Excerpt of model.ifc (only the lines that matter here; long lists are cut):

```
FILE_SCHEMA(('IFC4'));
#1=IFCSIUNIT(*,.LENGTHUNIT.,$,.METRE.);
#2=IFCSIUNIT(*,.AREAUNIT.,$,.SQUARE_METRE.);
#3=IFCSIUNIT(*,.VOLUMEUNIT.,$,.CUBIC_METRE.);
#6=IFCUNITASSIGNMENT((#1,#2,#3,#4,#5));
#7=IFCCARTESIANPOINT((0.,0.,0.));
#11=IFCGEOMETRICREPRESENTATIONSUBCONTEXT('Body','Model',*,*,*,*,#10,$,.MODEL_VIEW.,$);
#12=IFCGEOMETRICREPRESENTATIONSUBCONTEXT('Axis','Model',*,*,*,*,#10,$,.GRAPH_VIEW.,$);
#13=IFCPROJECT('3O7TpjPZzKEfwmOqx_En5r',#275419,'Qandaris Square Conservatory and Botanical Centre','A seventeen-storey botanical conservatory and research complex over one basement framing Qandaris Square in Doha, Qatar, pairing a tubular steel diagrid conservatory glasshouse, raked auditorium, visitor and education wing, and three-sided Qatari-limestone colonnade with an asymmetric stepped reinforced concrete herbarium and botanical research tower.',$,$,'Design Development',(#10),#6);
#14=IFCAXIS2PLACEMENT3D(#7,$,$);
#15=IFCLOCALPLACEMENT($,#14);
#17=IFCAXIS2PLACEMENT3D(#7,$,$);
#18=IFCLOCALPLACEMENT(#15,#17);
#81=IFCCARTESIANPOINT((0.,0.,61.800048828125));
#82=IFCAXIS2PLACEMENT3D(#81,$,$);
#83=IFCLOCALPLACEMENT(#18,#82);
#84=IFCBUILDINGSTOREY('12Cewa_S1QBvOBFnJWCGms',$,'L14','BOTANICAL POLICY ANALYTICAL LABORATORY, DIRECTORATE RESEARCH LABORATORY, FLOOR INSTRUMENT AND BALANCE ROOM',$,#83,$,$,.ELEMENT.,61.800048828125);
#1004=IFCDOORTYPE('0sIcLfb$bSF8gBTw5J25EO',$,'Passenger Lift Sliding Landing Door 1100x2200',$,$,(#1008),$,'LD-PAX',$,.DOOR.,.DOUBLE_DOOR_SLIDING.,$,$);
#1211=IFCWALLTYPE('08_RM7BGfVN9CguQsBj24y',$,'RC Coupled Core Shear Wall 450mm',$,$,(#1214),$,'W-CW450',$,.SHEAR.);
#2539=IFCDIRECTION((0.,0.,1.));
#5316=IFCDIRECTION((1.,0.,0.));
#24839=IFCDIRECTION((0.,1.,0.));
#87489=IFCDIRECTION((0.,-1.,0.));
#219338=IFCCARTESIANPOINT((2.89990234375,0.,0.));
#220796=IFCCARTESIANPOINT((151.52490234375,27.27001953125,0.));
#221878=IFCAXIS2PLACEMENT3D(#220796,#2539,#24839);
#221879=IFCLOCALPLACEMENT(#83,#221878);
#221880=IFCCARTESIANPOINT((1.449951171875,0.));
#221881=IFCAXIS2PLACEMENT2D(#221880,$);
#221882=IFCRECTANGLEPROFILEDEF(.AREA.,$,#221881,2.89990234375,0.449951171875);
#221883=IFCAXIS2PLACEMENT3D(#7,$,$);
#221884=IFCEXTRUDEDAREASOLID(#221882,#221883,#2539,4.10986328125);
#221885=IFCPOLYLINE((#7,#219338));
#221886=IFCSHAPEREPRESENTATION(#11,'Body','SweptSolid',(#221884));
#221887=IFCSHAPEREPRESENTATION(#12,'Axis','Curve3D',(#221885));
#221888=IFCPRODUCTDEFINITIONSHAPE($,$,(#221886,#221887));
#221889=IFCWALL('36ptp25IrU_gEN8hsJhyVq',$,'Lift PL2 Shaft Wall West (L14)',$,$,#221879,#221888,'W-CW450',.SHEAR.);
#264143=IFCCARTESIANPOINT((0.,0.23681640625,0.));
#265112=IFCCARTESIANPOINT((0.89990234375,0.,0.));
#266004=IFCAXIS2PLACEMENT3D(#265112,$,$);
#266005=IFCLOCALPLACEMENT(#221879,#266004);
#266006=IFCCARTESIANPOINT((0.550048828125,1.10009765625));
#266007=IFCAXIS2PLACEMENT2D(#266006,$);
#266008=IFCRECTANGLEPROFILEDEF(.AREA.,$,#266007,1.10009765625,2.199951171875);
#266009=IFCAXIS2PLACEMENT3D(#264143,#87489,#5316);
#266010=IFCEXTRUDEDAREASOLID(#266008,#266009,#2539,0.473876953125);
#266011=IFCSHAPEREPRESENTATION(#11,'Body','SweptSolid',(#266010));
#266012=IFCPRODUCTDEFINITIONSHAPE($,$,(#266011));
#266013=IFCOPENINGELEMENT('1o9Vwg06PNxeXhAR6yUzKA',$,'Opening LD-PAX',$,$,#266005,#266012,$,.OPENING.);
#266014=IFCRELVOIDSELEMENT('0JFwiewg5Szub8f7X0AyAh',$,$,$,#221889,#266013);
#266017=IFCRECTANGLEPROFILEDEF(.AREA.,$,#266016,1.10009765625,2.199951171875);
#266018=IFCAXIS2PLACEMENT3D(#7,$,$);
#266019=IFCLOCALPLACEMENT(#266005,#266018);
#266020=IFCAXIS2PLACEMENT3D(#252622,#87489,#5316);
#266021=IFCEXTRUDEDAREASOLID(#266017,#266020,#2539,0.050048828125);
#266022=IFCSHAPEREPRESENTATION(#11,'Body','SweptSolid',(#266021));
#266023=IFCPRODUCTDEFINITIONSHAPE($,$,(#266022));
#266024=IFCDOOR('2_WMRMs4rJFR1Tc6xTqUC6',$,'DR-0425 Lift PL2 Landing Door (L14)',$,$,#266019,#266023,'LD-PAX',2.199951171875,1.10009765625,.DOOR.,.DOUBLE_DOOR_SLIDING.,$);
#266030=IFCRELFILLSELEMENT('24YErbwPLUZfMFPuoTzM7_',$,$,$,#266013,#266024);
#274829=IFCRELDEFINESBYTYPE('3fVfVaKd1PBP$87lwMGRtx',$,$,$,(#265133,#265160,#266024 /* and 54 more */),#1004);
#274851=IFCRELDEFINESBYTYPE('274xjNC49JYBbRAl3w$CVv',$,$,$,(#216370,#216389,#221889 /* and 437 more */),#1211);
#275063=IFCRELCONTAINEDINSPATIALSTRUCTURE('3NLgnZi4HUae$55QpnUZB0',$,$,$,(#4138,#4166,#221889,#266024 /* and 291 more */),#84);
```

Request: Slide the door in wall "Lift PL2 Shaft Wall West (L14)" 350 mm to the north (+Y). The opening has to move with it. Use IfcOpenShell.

```python
import ifcopenshell
import ifcopenshell.api.geometry
import ifcopenshell.util.placement

model = ifcopenshell.open("model.ifc")

door = model.by_guid("2_WMRMs4rJFR1Tc6xTqUC6")
opening = door.FillsVoids[0].RelatingOpeningElement
wall = opening.VoidsElements[0].RelatingBuildingElement

wall_matrix = ifcopenshell.util.placement.get_local_placement(wall.ObjectPlacement)
shift = wall_matrix[:3, 0] * 0.35
before = ifcopenshell.util.placement.get_local_placement(door.ObjectPlacement)[:3, 3].copy()

# The door is placed relative to its opening, so it follows when the opening moves.
matrix = ifcopenshell.util.placement.get_local_placement(opening.ObjectPlacement)
matrix[:3, 3] += shift
ifcopenshell.api.geometry.edit_object_placement(
    model, product=opening, matrix=matrix, is_si=False, should_transform_children=True
)

after = ifcopenshell.util.placement.get_local_placement(door.ObjectPlacement)[:3, 3]
print("door moved by", (after - before).round(3) + 0.0)

model.write("model_updated.ifc")
```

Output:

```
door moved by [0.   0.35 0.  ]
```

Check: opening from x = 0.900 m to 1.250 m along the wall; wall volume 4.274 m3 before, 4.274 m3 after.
